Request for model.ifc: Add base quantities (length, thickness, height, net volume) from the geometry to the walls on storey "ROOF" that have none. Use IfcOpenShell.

First a look at what the model holds.

```python
import ifcopenshell
import ifcopenshell.util.element
import ifcopenshell.util.unit

model = ifcopenshell.open("model.ifc")
print(model.schema)
for unit_type in ("LENGTHUNIT", "AREAUNIT", "VOLUMEUNIT"):
    print(unit_type, ifcopenshell.util.unit.calculate_unit_scale(model, unit_type))
storey = next(s for s in model.by_type("IfcBuildingStorey") if s.Name == "ROOF")
walls = [e for e in ifcopenshell.util.element.get_decomposition(storey) if e.is_a("IfcWall")]
for e in sorted(walls, key=lambda e: e.id()):
    print(e.id(), e.is_a(), e.Name, list(ifcopenshell.util.element.get_psets(e, qtos_only=True)), sep=" | ")
```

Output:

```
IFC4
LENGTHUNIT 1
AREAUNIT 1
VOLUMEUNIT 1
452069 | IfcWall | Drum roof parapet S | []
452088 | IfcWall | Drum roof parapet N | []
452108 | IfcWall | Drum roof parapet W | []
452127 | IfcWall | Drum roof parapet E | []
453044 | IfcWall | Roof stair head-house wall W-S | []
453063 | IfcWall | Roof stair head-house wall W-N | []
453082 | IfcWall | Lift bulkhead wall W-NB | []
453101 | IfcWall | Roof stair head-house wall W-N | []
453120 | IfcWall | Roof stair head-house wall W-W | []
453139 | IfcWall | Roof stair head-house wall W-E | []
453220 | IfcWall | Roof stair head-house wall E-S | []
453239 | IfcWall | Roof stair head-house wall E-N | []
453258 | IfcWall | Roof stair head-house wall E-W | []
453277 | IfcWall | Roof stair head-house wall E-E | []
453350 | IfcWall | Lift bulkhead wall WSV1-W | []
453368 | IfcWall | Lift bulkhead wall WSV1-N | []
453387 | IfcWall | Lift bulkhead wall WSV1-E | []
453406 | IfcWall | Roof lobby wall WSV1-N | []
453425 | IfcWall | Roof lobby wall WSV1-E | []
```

```python
import ifcopenshell
import ifcopenshell.api.pset
import ifcopenshell.geom
import ifcopenshell.util.element
import ifcopenshell.util.shape
import ifcopenshell.util.unit

model = ifcopenshell.open("model.ifc")
unit_scale = ifcopenshell.util.unit.calculate_unit_scale(model)
volume_scale = ifcopenshell.util.unit.calculate_unit_scale(model, "VOLUMEUNIT")
settings = ifcopenshell.geom.settings()

storey = next(s for s in model.by_type("IfcBuildingStorey") if s.Name == "ROOF")
walls = [e for e in ifcopenshell.util.element.get_decomposition(storey) if e.is_a("IfcWall")]

for e in sorted(walls, key=lambda e: e.id()):
    if ifcopenshell.util.element.get_psets(e, qtos_only=True, should_inherit=False):
        continue
    # Geometry comes back in metres, in the element's own axes.
    shape = ifcopenshell.geom.create_shape(settings, e)
    values = {
        "Length": ifcopenshell.util.shape.get_x(shape.geometry) / unit_scale,
        "Width": ifcopenshell.util.shape.get_y(shape.geometry) / unit_scale,
        "Height": ifcopenshell.util.shape.get_z(shape.geometry) / unit_scale,
        "NetVolume": ifcopenshell.util.shape.get_volume(shape.geometry) / volume_scale,
    }
    qto = ifcopenshell.api.pset.add_qto(model, product=e, name="Qto_WallBaseQuantities")
    ifcopenshell.api.pset.edit_qto(model, qto=qto, properties=values)
    print(e.id(), {k: round(v, 3) for k, v in values.items()})

model.write("model_rev.ifc")
```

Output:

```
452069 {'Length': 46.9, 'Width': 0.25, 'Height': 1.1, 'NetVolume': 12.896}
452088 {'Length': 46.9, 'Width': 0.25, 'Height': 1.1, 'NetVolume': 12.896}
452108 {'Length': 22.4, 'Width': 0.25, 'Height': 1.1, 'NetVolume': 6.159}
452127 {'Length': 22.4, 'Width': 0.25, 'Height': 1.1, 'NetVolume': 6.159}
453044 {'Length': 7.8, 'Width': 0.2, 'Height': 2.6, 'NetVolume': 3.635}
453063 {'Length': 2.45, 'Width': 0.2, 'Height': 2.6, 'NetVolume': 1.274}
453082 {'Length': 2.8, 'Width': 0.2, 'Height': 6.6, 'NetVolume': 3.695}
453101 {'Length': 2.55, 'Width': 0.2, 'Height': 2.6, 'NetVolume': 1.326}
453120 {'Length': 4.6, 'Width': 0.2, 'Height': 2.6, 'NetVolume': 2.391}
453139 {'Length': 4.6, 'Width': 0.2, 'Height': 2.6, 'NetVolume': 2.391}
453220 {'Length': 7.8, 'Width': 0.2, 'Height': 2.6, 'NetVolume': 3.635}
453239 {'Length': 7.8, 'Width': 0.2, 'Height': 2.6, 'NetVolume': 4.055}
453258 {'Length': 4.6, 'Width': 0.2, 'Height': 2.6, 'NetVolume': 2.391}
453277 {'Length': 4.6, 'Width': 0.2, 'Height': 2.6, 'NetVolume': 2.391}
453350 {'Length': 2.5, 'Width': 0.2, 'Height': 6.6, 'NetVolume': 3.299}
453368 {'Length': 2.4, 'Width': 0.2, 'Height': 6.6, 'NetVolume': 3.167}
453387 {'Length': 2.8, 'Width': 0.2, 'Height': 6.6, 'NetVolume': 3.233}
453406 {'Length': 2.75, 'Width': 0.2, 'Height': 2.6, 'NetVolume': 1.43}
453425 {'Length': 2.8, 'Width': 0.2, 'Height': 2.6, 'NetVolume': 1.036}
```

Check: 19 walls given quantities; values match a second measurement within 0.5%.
